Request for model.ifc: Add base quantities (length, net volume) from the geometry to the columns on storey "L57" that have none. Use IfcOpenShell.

First a look at what the model holds.

```python
import ifcopenshell
import ifcopenshell.util.element
import ifcopenshell.util.unit

model = ifcopenshell.open("model.ifc")
print(model.schema)
for unit_type in ("LENGTHUNIT", "AREAUNIT", "VOLUMEUNIT"):
    print(unit_type, ifcopenshell.util.unit.calculate_unit_scale(model, unit_type))
storey = next(s for s in model.by_type("IfcBuildingStorey") if s.Name == "L57")
columns = [e for e in ifcopenshell.util.element.get_decomposition(storey) if e.is_a("IfcColumn")]
for e in sorted(columns, key=lambda e: e.id()):
    print(e.id(), e.is_a(), e.Name, list(ifcopenshell.util.element.get_psets(e, qtos_only=True)), sep=" | ")
```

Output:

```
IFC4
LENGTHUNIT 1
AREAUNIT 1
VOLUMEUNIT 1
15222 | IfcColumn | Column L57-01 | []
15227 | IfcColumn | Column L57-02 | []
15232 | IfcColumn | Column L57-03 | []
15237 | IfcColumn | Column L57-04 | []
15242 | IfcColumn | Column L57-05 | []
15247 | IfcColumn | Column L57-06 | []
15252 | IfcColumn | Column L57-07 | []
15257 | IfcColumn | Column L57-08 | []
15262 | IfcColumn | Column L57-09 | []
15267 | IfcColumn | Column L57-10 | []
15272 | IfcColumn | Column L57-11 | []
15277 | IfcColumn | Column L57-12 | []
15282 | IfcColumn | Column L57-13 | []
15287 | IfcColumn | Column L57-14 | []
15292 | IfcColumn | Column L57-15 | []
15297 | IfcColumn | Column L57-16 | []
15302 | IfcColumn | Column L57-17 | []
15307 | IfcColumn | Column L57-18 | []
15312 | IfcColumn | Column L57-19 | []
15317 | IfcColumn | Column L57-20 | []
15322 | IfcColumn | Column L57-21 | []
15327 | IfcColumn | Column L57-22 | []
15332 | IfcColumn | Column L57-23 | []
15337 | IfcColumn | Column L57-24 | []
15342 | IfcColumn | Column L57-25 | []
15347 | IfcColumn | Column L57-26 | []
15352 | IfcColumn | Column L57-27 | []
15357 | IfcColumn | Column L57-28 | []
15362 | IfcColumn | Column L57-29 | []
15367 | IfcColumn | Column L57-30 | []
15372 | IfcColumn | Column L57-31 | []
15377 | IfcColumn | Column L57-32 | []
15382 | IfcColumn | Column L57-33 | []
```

```python
import ifcopenshell
import ifcopenshell.api.pset
import ifcopenshell.geom
import ifcopenshell.util.element
import ifcopenshell.util.shape
import ifcopenshell.util.unit

model = ifcopenshell.open("model.ifc")
unit_scale = ifcopenshell.util.unit.calculate_unit_scale(model)
volume_scale = ifcopenshell.util.unit.calculate_unit_scale(model, "VOLUMEUNIT")
settings = ifcopenshell.geom.settings()

storey = next(s for s in model.by_type("IfcBuildingStorey") if s.Name == "L57")
columns = [e for e in ifcopenshell.util.element.get_decomposition(storey) if e.is_a("IfcColumn")]

for e in sorted(columns, key=lambda e: e.id()):
    if ifcopenshell.util.element.get_psets(e, qtos_only=True, should_inherit=False):
        continue
    # Geometry comes back in metres, in the element's own axes.
    shape = ifcopenshell.geom.create_shape(settings, e)
    values = {
        "Length": ifcopenshell.util.shape.get_z(shape.geometry) / unit_scale,
        "NetVolume": ifcopenshell.util.shape.get_volume(shape.geometry) / volume_scale,
    }
    qto = ifcopenshell.api.pset.add_qto(model, product=e, name="Qto_ColumnBaseQuantities")
    ifcopenshell.api.pset.edit_qto(model, qto=qto, properties=values)
    print(e.id(), {k: round(v, 3) for k, v in values.items()})

model.write("model-out.ifc")
```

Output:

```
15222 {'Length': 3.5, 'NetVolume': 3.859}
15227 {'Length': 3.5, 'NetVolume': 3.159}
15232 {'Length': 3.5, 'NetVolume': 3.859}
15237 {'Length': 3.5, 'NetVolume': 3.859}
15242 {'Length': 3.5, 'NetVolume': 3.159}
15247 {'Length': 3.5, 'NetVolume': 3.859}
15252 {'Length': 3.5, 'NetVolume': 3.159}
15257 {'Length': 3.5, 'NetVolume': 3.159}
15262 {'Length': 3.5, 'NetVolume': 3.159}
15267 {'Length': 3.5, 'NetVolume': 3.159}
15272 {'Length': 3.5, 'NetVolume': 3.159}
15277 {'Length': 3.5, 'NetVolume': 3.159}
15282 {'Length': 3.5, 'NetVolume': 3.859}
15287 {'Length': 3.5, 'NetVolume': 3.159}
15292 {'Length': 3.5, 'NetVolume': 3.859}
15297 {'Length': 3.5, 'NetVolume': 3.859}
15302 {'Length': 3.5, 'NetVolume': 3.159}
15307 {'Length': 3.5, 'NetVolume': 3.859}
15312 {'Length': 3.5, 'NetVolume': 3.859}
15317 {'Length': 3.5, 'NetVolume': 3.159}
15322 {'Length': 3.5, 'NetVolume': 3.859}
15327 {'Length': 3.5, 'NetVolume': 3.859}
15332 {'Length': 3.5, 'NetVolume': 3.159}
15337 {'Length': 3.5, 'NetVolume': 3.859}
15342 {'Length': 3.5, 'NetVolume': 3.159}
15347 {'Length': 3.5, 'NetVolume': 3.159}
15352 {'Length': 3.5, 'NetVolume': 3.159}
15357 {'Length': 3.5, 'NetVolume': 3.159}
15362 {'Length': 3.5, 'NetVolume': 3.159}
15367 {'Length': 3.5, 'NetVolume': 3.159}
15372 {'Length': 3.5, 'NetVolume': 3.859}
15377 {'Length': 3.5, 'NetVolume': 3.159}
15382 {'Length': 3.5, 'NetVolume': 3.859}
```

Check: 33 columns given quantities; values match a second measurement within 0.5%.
